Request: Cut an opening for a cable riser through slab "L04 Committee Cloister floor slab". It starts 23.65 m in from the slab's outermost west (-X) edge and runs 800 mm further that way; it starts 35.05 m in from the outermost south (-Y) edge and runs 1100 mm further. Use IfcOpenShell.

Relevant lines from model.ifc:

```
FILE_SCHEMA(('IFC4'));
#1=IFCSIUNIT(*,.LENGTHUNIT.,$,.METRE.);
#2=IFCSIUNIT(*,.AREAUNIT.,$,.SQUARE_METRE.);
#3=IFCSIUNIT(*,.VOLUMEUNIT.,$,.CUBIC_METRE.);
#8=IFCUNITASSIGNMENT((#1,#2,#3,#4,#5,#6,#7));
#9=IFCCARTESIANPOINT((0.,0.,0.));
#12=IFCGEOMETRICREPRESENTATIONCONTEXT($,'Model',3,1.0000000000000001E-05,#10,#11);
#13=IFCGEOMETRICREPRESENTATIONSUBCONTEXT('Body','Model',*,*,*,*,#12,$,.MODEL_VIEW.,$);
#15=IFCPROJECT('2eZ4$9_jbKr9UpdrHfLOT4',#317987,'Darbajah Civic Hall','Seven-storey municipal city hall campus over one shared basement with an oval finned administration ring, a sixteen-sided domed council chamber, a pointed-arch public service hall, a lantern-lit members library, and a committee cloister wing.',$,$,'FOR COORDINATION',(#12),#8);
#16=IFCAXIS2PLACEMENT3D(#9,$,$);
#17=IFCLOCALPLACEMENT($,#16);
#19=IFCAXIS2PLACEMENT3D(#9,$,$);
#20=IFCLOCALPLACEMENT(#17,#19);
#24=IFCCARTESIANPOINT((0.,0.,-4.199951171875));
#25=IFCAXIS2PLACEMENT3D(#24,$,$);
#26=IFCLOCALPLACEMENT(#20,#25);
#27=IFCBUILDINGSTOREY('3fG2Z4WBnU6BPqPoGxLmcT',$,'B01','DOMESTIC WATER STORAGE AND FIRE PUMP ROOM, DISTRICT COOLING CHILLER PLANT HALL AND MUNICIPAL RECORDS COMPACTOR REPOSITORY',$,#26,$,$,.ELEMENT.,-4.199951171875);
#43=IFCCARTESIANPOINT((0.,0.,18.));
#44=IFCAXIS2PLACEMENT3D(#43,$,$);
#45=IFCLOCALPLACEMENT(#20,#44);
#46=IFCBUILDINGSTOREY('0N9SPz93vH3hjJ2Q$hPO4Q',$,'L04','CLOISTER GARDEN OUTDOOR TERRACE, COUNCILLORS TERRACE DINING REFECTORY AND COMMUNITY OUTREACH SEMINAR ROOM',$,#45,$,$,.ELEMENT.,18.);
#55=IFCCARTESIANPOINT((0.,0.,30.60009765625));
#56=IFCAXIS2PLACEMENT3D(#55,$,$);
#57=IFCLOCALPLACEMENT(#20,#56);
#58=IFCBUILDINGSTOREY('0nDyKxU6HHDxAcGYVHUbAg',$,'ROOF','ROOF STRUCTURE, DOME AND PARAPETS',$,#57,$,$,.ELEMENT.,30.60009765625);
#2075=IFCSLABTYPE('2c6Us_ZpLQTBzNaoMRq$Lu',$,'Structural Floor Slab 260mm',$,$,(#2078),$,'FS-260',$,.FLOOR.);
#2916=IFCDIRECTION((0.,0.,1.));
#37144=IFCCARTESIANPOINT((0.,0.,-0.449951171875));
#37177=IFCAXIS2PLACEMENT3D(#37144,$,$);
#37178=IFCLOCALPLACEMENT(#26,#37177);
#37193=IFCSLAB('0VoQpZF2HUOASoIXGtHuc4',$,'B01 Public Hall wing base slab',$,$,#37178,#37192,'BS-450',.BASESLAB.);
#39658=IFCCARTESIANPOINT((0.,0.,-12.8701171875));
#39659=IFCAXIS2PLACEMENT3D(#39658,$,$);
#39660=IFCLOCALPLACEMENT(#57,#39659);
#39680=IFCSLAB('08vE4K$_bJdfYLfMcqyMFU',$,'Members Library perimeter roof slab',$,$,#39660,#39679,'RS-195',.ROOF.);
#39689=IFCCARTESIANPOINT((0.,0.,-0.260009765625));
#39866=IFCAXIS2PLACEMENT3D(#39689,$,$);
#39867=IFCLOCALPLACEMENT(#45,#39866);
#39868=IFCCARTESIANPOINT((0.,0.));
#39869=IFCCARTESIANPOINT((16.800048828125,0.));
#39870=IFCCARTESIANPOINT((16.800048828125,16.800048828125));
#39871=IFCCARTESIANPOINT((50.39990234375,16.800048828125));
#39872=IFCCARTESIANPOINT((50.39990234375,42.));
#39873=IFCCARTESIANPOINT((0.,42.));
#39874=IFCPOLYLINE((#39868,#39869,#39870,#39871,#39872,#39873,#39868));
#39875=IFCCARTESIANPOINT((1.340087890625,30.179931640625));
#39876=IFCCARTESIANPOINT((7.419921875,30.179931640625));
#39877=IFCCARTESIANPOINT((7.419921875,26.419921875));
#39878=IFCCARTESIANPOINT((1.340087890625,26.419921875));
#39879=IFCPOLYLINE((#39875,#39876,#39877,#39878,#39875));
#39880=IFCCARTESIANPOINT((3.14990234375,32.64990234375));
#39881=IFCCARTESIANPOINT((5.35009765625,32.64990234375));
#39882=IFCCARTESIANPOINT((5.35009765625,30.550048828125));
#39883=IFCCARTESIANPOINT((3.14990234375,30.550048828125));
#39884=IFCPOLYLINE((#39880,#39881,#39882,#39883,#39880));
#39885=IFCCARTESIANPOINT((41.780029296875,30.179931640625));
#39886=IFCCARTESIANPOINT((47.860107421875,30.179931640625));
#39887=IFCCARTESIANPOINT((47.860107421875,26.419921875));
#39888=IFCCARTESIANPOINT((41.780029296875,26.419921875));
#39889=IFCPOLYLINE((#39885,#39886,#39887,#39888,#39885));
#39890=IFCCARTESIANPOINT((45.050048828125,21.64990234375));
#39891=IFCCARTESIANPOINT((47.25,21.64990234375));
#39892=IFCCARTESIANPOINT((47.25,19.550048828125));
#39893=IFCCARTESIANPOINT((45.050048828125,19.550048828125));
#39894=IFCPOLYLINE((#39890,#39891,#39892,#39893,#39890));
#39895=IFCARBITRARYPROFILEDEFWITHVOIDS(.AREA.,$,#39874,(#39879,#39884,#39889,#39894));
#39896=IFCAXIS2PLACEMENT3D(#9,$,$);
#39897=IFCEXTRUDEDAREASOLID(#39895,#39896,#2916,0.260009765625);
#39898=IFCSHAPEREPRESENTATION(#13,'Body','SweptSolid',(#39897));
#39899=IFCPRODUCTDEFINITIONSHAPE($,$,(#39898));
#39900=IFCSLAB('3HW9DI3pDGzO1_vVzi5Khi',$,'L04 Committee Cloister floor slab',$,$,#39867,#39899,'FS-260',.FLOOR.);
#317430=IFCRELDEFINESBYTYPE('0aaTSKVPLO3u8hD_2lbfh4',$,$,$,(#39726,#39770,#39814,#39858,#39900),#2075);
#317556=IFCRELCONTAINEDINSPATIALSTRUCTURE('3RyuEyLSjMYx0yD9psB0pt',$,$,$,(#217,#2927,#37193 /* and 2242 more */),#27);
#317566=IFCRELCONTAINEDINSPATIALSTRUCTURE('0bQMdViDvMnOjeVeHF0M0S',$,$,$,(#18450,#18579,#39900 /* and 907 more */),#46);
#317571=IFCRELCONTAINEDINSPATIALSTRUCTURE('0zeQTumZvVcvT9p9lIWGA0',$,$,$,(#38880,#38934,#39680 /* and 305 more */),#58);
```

```python
import numpy as np
import ifcopenshell
import ifcopenshell.api.feature
import ifcopenshell.api.geometry
import ifcopenshell.api.root
import ifcopenshell.geom
import ifcopenshell.util.placement
import ifcopenshell.util.representation
import ifcopenshell.util.shape
import ifcopenshell.util.unit

model = ifcopenshell.open("model.ifc")
unit_scale = ifcopenshell.util.unit.calculate_unit_scale(model)
settings = ifcopenshell.geom.settings()


def volume(element):
    """Net volume in cubic metres, openings subtracted."""
    shape = ifcopenshell.geom.create_shape(settings, element)
    return ifcopenshell.util.shape.get_volume(shape.geometry)


slab = model.by_guid("3HW9DI3pDGzO1_vVzi5Khi")
before = volume(slab)

# Extent in the slab's own axes, in metres. The edges named are its -X and -Y sides.
slab_shape = ifcopenshell.geom.create_shape(settings, slab)
vertices = ifcopenshell.util.shape.get_vertices(slab_shape.geometry)
x_min, y_min, bottom = vertices.min(axis=0)
top = vertices[:, 2].max()

opening = ifcopenshell.api.root.create_entity(model, ifc_class="IfcOpeningElement", name="Cable riser opening", predefined_type="OPENING")
context = ifcopenshell.util.representation.get_context(model, "Model", "Body", "MODEL_VIEW")
width, depth = 0.8, 1.1
outline = [(0.0, 0.0), (width, 0.0), (width, depth), (0.0, depth), (0.0, 0.0)]
# Overshoot both faces by 50 mm so the cut is clean.
shape = ifcopenshell.api.geometry.add_slab_representation(
    model, context=context, depth=top - bottom + 0.1, polyline=outline
)
ifcopenshell.api.geometry.assign_representation(model, product=opening, representation=shape)

matrix = ifcopenshell.util.placement.get_local_placement(slab.ObjectPlacement)
matrix[:, 3] = matrix @ np.append(np.array([x_min + 23.65, y_min + 35.05, bottom - 0.05]) / unit_scale, 1.0)
ifcopenshell.api.geometry.edit_object_placement(model, product=opening, matrix=matrix, is_si=False)
ifcopenshell.api.feature.add_feature(model, feature=opening, element=slab)

after = volume(slab)

print(f"slab volume {before:.3f} -> {after:.3f} m3")

model.write("model_edited.ifc")
```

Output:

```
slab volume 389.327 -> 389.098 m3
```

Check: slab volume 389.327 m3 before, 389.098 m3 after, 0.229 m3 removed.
